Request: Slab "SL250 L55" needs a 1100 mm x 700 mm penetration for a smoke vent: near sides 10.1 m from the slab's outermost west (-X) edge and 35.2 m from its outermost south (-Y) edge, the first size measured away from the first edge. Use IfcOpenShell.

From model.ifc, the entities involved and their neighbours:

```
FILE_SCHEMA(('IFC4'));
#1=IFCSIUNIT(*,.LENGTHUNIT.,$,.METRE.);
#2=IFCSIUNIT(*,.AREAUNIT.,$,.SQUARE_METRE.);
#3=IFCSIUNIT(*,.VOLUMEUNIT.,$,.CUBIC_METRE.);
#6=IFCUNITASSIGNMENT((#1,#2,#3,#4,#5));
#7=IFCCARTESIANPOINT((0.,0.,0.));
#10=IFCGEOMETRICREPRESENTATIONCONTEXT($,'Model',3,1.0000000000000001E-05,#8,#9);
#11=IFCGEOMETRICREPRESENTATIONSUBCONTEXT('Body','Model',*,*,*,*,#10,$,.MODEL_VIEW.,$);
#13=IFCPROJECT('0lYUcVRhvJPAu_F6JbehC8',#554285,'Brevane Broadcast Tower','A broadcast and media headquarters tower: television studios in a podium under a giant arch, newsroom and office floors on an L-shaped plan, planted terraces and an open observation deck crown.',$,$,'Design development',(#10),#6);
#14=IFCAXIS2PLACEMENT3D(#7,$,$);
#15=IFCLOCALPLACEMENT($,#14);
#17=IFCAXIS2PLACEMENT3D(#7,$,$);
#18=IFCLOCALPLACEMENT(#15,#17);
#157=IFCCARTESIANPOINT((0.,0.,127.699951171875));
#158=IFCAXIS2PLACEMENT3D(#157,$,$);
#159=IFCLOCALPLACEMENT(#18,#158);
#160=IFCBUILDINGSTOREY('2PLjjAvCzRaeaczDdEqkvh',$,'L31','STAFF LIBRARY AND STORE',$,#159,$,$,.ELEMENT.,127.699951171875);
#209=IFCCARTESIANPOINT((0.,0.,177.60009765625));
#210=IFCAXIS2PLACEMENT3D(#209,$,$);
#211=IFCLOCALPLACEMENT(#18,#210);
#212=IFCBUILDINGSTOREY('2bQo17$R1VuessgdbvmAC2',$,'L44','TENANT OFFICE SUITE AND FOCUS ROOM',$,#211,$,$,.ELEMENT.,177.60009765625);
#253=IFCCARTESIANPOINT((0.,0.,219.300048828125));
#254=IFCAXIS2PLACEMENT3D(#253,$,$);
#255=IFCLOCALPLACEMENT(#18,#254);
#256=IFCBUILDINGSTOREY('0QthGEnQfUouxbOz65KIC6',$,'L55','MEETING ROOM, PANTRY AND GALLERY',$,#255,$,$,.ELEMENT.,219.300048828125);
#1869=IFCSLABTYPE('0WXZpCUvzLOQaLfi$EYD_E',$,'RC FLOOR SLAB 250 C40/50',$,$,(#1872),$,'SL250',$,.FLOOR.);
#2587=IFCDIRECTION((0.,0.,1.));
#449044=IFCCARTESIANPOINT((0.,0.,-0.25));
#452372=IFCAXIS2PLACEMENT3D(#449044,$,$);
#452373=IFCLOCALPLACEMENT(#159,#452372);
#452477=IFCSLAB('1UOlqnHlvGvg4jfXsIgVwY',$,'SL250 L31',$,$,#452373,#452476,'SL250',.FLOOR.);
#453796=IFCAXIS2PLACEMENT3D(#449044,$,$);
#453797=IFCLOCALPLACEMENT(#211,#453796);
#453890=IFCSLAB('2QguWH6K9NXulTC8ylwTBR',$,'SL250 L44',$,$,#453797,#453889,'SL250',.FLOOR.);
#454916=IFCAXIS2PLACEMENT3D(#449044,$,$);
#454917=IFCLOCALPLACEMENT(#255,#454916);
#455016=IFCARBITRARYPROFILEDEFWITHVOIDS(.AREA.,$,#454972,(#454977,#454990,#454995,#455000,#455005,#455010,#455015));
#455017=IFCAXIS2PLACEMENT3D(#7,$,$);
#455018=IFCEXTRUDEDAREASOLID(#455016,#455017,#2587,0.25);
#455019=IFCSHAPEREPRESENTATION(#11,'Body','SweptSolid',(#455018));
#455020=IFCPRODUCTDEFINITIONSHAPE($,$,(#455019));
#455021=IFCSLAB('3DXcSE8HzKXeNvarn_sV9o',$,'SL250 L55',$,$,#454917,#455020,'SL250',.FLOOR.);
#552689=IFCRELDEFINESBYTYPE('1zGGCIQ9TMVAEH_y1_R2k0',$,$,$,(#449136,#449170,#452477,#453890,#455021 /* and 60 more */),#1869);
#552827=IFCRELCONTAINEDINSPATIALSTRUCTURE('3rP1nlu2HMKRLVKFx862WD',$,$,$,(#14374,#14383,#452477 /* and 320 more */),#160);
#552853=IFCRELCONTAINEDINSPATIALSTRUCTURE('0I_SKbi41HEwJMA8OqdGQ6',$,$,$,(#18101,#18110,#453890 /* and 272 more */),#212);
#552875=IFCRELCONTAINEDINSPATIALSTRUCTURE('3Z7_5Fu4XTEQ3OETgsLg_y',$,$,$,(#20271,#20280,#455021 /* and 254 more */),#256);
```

```python
import numpy as np
import ifcopenshell
import ifcopenshell.api.feature
import ifcopenshell.api.geometry
import ifcopenshell.api.root
import ifcopenshell.geom
import ifcopenshell.util.placement
import ifcopenshell.util.representation
import ifcopenshell.util.shape
import ifcopenshell.util.unit

model = ifcopenshell.open("model.ifc")
unit_scale = ifcopenshell.util.unit.calculate_unit_scale(model)
settings = ifcopenshell.geom.settings()


def volume(element):
    """Net volume in cubic metres, openings subtracted."""
    shape = ifcopenshell.geom.create_shape(settings, element)
    return ifcopenshell.util.shape.get_volume(shape.geometry)


slab = model.by_id(455021)
before = volume(slab)

# Extent in the slab's own axes, in metres. The edges named are its -X and -Y sides.
slab_shape = ifcopenshell.geom.create_shape(settings, slab)
vertices = ifcopenshell.util.shape.get_vertices(slab_shape.geometry)
x_min, y_min, bottom = vertices.min(axis=0)
top = vertices[:, 2].max()

opening = ifcopenshell.api.root.create_entity(model, ifc_class="IfcOpeningElement", name="Smoke vent opening", predefined_type="OPENING")
context = ifcopenshell.util.representation.get_context(model, "Model", "Body", "MODEL_VIEW")
width, depth = 1.1, 0.7
outline = [(0.0, 0.0), (width, 0.0), (width, depth), (0.0, depth), (0.0, 0.0)]
# Overshoot both faces by 50 mm so the cut is clean.
shape = ifcopenshell.api.geometry.add_slab_representation(
    model, context=context, depth=top - bottom + 0.1, polyline=outline
)
ifcopenshell.api.geometry.assign_representation(model, product=opening, representation=shape)

matrix = ifcopenshell.util.placement.get_local_placement(slab.ObjectPlacement)
matrix[:, 3] = matrix @ np.append(np.array([x_min + 10.1, y_min + 35.2, bottom - 0.05]) / unit_scale, 1.0)
ifcopenshell.api.geometry.edit_object_placement(model, product=opening, matrix=matrix, is_si=False)
ifcopenshell.api.feature.add_feature(model, feature=opening, element=slab)

after = volume(slab)

print(f"slab volume {before:.3f} -> {after:.3f} m3")

model.write("model_updated.ifc")
```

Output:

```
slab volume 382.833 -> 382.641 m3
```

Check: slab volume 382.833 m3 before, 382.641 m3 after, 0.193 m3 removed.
